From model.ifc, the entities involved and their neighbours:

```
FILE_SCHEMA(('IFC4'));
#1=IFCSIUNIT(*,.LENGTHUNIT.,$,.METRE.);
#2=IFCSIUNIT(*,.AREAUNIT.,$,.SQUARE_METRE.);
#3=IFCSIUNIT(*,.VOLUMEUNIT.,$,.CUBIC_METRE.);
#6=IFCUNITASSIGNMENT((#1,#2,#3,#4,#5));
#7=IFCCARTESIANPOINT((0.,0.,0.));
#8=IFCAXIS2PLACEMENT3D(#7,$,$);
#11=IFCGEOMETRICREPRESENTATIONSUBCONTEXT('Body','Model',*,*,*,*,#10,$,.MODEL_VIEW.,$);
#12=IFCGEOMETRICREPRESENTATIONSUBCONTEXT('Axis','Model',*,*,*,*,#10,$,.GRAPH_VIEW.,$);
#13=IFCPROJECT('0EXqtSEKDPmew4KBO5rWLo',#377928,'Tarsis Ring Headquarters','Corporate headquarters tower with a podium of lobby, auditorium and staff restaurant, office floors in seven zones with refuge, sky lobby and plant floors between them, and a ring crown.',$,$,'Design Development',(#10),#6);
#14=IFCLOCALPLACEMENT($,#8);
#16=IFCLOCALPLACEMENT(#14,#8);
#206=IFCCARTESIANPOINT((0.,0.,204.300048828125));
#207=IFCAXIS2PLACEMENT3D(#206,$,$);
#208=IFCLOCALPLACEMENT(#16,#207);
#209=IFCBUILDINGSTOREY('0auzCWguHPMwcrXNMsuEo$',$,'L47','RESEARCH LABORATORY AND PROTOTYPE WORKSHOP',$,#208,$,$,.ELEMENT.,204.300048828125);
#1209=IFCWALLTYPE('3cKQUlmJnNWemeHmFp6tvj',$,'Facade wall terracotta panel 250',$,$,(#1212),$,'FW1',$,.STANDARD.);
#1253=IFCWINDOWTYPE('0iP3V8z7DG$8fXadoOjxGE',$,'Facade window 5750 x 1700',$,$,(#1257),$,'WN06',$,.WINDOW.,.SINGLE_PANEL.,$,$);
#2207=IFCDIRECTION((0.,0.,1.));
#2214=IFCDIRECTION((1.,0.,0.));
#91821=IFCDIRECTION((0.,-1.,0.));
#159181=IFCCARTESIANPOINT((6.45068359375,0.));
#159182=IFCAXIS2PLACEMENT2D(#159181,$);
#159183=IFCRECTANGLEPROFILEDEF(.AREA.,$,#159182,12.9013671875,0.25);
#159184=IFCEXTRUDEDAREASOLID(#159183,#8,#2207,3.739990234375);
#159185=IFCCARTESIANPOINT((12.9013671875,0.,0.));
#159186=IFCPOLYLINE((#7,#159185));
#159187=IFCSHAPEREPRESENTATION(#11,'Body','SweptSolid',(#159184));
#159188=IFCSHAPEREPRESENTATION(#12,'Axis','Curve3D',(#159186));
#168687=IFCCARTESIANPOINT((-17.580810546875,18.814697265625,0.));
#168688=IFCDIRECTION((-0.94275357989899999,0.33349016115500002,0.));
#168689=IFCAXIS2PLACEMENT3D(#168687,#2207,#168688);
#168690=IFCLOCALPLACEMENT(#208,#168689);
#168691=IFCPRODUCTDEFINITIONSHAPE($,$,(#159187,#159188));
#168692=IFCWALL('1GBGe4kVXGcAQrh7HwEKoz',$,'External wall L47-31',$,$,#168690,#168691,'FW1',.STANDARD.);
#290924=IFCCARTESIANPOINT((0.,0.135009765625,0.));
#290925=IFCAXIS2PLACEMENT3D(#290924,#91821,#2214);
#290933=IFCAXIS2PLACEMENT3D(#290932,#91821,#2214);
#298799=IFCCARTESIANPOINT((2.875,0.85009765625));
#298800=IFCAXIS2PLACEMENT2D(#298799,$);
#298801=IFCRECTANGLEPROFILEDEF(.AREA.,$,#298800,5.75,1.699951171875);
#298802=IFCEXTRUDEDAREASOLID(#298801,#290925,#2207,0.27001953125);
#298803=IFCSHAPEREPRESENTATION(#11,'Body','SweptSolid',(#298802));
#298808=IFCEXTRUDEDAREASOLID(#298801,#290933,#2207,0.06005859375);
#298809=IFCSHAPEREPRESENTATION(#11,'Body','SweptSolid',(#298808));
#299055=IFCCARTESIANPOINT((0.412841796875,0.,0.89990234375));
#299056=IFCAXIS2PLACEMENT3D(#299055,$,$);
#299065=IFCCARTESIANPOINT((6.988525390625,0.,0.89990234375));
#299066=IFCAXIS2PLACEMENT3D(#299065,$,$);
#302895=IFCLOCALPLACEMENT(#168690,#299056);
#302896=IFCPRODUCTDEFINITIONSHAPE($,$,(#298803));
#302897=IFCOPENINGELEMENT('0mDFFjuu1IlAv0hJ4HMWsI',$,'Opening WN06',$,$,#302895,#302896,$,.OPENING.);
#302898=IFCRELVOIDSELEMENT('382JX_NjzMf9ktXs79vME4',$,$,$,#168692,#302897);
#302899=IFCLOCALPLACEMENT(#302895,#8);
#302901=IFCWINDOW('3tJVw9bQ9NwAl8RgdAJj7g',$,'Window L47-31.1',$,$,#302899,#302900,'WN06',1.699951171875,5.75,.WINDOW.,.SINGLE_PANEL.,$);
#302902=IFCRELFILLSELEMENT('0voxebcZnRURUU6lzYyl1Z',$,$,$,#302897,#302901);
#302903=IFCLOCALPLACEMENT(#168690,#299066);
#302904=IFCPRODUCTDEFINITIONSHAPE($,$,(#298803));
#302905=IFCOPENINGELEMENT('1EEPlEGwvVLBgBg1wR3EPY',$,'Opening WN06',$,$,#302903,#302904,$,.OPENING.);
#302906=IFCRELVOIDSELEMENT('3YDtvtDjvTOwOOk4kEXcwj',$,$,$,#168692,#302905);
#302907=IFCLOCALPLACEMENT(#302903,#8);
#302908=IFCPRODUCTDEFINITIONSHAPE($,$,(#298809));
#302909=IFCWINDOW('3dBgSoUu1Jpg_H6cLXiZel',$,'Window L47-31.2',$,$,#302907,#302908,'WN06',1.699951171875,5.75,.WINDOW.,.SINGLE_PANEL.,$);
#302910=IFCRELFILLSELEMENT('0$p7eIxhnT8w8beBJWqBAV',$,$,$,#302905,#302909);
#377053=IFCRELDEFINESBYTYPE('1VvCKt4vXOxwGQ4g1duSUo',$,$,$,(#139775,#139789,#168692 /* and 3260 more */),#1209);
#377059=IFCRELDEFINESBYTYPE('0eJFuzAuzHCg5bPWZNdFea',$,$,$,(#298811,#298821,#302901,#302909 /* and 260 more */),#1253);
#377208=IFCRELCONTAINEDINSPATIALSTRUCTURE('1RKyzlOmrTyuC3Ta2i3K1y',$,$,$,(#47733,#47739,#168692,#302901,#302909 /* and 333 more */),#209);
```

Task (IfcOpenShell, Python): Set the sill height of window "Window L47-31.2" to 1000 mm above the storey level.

```python
import numpy as np
import ifcopenshell
import ifcopenshell.api.geometry
import ifcopenshell.geom
import ifcopenshell.util.element
import ifcopenshell.util.placement
import ifcopenshell.util.shape
import ifcopenshell.util.unit

model = ifcopenshell.open("model.ifc")
unit_scale = ifcopenshell.util.unit.calculate_unit_scale(model)

window = model.by_guid("3dBgSoUu1Jpg_H6cLXiZel")
opening = window.FillsVoids[0].RelatingOpeningElement
storey = ifcopenshell.util.element.get_container(window, ifc_class="IfcBuildingStorey")
level = ifcopenshell.util.placement.get_local_placement(storey.ObjectPlacement)[2, 3]

# The opening's origin need not be at the sill, so measure its lowest point.
shape = ifcopenshell.geom.create_shape(ifcopenshell.geom.settings(), opening)
bottom = ifcopenshell.util.shape.get_shape_bottom_elevation(shape, shape.geometry) / unit_scale
dz = level + 1 / unit_scale - bottom

shift = np.array([0.0, 0.0, dz])
# The window is placed relative to its opening, so it follows when the opening moves.
matrix = ifcopenshell.util.placement.get_local_placement(opening.ObjectPlacement)
matrix[:3, 3] += shift
ifcopenshell.api.geometry.edit_object_placement(
    model, product=opening, matrix=matrix, is_si=False, should_transform_children=True
)

print(f"moved by {dz * unit_scale:+.3f} m")

model.write("model_rev.ifc")
```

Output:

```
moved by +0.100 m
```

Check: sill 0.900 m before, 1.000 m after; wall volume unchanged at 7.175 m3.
